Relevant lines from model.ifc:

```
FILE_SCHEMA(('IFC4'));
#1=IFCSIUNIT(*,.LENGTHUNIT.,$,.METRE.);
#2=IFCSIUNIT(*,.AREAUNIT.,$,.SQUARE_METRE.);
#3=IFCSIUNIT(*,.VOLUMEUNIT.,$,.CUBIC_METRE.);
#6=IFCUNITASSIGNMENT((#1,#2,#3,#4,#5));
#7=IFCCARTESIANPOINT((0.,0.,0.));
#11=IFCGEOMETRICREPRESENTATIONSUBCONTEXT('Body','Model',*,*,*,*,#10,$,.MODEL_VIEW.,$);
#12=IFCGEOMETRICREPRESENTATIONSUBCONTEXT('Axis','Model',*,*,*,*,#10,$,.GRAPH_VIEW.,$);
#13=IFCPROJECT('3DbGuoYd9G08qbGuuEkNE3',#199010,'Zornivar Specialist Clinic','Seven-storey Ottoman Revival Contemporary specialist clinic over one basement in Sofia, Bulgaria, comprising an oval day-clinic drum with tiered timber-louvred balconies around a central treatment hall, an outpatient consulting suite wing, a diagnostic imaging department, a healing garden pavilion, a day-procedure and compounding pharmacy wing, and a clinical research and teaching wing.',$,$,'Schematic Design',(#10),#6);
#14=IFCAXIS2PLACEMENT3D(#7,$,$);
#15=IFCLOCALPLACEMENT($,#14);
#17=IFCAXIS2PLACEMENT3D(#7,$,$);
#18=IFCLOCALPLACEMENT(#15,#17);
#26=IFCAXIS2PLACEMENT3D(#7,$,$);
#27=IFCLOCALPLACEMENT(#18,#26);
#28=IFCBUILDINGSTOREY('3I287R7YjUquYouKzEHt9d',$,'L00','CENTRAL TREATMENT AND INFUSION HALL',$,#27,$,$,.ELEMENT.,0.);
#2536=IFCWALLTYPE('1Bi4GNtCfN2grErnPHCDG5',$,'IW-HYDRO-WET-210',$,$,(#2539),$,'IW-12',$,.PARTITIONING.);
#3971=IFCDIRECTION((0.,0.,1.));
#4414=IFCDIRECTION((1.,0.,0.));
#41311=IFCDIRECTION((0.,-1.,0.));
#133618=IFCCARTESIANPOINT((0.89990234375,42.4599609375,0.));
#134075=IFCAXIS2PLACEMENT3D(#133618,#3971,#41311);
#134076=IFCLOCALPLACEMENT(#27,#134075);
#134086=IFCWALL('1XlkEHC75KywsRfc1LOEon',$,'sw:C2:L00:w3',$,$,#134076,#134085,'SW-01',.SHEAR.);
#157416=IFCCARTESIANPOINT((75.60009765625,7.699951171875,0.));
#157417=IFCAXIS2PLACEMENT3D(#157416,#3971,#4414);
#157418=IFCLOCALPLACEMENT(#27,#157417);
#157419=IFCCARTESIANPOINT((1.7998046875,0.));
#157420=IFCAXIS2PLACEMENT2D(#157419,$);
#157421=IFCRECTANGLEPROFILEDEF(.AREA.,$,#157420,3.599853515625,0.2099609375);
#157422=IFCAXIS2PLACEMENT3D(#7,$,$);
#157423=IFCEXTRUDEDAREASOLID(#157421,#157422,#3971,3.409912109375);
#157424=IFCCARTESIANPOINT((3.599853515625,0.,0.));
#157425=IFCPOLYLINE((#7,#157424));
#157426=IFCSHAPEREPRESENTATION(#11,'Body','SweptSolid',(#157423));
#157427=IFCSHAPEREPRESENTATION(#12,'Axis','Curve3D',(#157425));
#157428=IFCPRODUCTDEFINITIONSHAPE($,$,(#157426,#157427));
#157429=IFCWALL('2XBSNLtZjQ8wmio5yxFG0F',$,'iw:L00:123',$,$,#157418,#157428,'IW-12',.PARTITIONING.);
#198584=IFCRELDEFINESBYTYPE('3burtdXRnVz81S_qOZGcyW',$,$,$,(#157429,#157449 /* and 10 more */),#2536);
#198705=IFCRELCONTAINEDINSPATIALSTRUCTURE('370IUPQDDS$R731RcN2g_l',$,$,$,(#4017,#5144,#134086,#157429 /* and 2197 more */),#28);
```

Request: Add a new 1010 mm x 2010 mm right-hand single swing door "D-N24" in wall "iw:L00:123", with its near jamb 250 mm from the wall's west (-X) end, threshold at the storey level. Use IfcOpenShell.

```python
import numpy as np
import ifcopenshell
import ifcopenshell.api.feature
import ifcopenshell.api.geometry
import ifcopenshell.api.root
import ifcopenshell.api.spatial
import ifcopenshell.geom
import ifcopenshell.util.element
import ifcopenshell.util.placement
import ifcopenshell.util.representation
import ifcopenshell.util.shape
import ifcopenshell.util.unit

model = ifcopenshell.open("model.ifc")
unit_scale = ifcopenshell.util.unit.calculate_unit_scale(model)
settings = ifcopenshell.geom.settings()


def volume(element):
    """Net volume in cubic metres, openings subtracted."""
    shape = ifcopenshell.geom.create_shape(settings, element)
    return ifcopenshell.util.shape.get_volume(shape.geometry)


wall = model.by_guid("2XBSNLtZjQ8wmio5yxFG0F")
storey = ifcopenshell.util.element.get_container(wall, ifc_class="IfcBuildingStorey")
context = ifcopenshell.util.representation.get_context(model, "Model", "Body", "MODEL_VIEW")
before = volume(wall)

width, height, from_end, sill = 1.01, 2.01, 0.25, 0.0  # metres

# The wall runs along its own X axis, and the end named is its -X end.
wall_shape = ifcopenshell.geom.create_shape(settings, wall)
x, y, z = ifcopenshell.util.shape.get_vertices(wall_shape.geometry).T
start = x.min() + from_end
face, thickness = float(y.min()), float(y.max() - y.min())
wall_matrix = ifcopenshell.util.placement.get_local_placement(wall.ObjectPlacement)
level = ifcopenshell.util.placement.get_local_placement(storey.ObjectPlacement)[2, 3]


def in_wall(x, y):
    """Placement at x, y metres in the wall's axes, at sill height."""
    matrix = wall_matrix.copy()
    matrix[:, 3] = wall_matrix @ np.array([x / unit_scale, y / unit_scale, 0.0, 1.0])
    matrix[2, 3] = level + sill / unit_scale
    return matrix


# Opening: a box that overshoots both wall faces by 50 mm.
opening = ifcopenshell.api.root.create_entity(model, ifc_class="IfcOpeningElement", predefined_type="OPENING")
box = ifcopenshell.api.geometry.add_wall_representation(
    model, context=context, length=width, height=height, thickness=thickness + 0.1
)
ifcopenshell.api.geometry.assign_representation(model, product=opening, representation=box)
ifcopenshell.api.geometry.edit_object_placement(model, product=opening, matrix=in_wall(start, face - 0.05), is_si=False)
ifcopenshell.api.feature.add_feature(model, feature=opening, element=wall)

door = ifcopenshell.api.root.create_entity(model, ifc_class="IfcDoor", name="D-N24", predefined_type="DOOR")
door.OverallWidth, door.OverallHeight = width / unit_scale, height / unit_scale
door.OperationType = "SINGLE_SWING_RIGHT"
body = ifcopenshell.api.geometry.add_door_representation(
    model,
    context=context,
    overall_width=door.OverallWidth,
    overall_height=door.OverallHeight,
    operation_type="SINGLE_SWING_RIGHT",
    lining_properties={"LiningDepth": thickness / unit_scale, "ThresholdDepth": thickness / unit_scale},
)
ifcopenshell.api.geometry.assign_representation(model, product=door, representation=body)
ifcopenshell.api.spatial.assign_container(model, products=[door], relating_structure=storey)
ifcopenshell.api.feature.add_filling(model, opening=opening, element=door)

# The lining spans the wall, so the door starts at the wall face.
ifcopenshell.api.geometry.edit_object_placement(model, product=door, matrix=in_wall(start, face), is_si=False)

after = volume(wall)

print(f"wall volume {before:.3f} -> {after:.3f} m3")

model.write("model_rev.ifc")
```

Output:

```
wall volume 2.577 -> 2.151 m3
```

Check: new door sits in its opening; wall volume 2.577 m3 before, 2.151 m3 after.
